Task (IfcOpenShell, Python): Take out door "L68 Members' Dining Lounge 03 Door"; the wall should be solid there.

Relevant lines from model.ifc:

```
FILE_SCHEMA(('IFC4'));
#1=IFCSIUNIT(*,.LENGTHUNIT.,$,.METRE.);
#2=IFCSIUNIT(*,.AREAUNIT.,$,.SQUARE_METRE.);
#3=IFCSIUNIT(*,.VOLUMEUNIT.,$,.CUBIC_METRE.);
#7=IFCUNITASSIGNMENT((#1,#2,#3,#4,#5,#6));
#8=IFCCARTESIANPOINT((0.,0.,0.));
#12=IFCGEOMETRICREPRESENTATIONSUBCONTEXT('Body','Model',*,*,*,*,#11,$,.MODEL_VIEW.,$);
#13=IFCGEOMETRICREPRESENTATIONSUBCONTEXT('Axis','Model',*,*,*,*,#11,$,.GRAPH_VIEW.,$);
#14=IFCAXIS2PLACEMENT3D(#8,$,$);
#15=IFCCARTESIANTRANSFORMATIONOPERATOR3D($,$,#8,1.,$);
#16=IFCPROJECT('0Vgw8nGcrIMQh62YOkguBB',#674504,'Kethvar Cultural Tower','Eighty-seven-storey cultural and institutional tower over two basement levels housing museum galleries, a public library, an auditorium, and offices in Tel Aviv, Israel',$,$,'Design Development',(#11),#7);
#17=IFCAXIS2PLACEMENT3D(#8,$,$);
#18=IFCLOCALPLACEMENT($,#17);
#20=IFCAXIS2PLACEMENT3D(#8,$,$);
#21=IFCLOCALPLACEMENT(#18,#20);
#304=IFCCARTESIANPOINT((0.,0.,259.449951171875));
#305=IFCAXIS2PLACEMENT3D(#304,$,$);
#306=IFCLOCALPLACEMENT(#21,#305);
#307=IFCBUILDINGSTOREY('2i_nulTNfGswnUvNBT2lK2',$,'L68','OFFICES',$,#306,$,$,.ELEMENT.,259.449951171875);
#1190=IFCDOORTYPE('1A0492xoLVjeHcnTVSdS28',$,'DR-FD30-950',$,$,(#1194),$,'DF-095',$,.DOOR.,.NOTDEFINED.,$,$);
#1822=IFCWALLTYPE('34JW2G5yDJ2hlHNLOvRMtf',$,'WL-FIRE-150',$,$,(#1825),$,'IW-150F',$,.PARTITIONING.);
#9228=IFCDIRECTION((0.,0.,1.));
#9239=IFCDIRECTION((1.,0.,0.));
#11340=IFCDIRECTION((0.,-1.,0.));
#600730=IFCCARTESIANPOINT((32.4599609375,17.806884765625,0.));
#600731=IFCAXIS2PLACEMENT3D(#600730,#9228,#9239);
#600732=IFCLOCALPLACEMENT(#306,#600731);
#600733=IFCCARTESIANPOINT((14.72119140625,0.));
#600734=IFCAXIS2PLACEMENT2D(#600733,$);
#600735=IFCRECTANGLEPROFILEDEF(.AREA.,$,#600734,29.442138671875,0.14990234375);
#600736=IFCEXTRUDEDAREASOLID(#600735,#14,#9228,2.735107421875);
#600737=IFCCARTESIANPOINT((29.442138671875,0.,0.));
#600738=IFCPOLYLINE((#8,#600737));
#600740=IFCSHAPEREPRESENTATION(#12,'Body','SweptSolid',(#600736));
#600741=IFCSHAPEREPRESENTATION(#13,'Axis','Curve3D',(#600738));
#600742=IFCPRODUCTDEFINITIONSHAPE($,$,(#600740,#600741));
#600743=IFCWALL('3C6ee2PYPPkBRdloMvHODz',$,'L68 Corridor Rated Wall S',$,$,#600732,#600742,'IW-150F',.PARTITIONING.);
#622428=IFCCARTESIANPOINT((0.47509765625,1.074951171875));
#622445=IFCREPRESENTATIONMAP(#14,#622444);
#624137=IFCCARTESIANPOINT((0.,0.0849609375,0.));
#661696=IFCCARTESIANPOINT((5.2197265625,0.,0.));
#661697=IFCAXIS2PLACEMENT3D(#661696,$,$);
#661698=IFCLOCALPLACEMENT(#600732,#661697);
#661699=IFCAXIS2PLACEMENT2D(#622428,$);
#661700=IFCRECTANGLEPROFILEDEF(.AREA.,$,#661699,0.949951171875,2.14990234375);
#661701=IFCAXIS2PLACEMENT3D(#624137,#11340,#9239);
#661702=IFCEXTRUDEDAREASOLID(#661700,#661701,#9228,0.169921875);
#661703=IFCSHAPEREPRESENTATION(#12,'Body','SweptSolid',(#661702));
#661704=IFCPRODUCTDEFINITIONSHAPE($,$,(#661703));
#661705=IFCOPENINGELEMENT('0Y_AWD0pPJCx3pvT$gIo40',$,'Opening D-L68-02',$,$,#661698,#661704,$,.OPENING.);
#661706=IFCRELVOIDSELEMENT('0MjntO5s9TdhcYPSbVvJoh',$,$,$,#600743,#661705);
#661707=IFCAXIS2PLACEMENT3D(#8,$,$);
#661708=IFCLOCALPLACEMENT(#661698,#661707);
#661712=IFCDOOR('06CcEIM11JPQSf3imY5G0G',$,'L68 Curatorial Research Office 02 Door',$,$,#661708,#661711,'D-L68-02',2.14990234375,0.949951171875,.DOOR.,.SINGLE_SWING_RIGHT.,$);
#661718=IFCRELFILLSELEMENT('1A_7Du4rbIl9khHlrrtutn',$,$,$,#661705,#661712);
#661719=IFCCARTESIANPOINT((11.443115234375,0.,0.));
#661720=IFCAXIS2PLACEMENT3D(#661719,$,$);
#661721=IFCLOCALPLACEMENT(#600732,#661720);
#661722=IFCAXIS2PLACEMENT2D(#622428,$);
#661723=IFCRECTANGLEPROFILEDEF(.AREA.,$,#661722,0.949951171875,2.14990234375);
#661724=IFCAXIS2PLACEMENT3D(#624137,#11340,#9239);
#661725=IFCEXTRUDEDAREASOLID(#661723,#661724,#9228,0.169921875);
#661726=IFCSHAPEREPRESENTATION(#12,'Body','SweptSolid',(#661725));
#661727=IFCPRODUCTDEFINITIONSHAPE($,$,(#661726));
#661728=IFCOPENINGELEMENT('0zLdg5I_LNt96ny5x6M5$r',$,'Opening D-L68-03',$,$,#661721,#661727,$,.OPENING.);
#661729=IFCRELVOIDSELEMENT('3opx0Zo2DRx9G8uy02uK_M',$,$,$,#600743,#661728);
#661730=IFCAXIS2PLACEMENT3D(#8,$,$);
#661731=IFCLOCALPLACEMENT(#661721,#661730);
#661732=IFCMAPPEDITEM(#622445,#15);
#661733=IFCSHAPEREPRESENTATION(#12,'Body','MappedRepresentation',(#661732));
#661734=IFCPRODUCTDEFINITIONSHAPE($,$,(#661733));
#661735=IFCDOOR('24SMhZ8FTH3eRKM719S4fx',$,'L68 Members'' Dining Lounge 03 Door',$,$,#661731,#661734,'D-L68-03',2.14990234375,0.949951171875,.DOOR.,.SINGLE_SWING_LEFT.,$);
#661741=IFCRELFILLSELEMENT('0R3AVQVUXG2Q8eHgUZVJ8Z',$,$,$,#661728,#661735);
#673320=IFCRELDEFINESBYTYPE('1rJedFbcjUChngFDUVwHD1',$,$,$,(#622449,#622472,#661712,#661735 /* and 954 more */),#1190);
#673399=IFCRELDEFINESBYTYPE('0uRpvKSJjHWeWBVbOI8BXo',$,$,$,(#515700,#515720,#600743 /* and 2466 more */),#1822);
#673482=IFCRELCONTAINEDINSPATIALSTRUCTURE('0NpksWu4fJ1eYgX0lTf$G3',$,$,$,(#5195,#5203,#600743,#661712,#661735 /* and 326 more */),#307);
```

```python
import ifcopenshell
import ifcopenshell.api.feature
import ifcopenshell.api.root
import ifcopenshell.geom
import ifcopenshell.util.shape

model = ifcopenshell.open("model.ifc")
settings = ifcopenshell.geom.settings()


def volume(element):
    """Net volume in cubic metres, openings subtracted."""
    shape = ifcopenshell.geom.create_shape(settings, element)
    return ifcopenshell.util.shape.get_volume(shape.geometry)


door = model.by_guid("24SMhZ8FTH3eRKM719S4fx")
opening = door.FillsVoids[0].RelatingOpeningElement
wall = opening.VoidsElements[0].RelatingBuildingElement
before = volume(wall)

ifcopenshell.api.root.remove_product(model, product=door)
ifcopenshell.api.feature.remove_feature(model, feature=opening)

after = volume(wall)

print(f"wall volume {before:.3f} -> {after:.3f} m3")

model.write("model_edited.ifc")
```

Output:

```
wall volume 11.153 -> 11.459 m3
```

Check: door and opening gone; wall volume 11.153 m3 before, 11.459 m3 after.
